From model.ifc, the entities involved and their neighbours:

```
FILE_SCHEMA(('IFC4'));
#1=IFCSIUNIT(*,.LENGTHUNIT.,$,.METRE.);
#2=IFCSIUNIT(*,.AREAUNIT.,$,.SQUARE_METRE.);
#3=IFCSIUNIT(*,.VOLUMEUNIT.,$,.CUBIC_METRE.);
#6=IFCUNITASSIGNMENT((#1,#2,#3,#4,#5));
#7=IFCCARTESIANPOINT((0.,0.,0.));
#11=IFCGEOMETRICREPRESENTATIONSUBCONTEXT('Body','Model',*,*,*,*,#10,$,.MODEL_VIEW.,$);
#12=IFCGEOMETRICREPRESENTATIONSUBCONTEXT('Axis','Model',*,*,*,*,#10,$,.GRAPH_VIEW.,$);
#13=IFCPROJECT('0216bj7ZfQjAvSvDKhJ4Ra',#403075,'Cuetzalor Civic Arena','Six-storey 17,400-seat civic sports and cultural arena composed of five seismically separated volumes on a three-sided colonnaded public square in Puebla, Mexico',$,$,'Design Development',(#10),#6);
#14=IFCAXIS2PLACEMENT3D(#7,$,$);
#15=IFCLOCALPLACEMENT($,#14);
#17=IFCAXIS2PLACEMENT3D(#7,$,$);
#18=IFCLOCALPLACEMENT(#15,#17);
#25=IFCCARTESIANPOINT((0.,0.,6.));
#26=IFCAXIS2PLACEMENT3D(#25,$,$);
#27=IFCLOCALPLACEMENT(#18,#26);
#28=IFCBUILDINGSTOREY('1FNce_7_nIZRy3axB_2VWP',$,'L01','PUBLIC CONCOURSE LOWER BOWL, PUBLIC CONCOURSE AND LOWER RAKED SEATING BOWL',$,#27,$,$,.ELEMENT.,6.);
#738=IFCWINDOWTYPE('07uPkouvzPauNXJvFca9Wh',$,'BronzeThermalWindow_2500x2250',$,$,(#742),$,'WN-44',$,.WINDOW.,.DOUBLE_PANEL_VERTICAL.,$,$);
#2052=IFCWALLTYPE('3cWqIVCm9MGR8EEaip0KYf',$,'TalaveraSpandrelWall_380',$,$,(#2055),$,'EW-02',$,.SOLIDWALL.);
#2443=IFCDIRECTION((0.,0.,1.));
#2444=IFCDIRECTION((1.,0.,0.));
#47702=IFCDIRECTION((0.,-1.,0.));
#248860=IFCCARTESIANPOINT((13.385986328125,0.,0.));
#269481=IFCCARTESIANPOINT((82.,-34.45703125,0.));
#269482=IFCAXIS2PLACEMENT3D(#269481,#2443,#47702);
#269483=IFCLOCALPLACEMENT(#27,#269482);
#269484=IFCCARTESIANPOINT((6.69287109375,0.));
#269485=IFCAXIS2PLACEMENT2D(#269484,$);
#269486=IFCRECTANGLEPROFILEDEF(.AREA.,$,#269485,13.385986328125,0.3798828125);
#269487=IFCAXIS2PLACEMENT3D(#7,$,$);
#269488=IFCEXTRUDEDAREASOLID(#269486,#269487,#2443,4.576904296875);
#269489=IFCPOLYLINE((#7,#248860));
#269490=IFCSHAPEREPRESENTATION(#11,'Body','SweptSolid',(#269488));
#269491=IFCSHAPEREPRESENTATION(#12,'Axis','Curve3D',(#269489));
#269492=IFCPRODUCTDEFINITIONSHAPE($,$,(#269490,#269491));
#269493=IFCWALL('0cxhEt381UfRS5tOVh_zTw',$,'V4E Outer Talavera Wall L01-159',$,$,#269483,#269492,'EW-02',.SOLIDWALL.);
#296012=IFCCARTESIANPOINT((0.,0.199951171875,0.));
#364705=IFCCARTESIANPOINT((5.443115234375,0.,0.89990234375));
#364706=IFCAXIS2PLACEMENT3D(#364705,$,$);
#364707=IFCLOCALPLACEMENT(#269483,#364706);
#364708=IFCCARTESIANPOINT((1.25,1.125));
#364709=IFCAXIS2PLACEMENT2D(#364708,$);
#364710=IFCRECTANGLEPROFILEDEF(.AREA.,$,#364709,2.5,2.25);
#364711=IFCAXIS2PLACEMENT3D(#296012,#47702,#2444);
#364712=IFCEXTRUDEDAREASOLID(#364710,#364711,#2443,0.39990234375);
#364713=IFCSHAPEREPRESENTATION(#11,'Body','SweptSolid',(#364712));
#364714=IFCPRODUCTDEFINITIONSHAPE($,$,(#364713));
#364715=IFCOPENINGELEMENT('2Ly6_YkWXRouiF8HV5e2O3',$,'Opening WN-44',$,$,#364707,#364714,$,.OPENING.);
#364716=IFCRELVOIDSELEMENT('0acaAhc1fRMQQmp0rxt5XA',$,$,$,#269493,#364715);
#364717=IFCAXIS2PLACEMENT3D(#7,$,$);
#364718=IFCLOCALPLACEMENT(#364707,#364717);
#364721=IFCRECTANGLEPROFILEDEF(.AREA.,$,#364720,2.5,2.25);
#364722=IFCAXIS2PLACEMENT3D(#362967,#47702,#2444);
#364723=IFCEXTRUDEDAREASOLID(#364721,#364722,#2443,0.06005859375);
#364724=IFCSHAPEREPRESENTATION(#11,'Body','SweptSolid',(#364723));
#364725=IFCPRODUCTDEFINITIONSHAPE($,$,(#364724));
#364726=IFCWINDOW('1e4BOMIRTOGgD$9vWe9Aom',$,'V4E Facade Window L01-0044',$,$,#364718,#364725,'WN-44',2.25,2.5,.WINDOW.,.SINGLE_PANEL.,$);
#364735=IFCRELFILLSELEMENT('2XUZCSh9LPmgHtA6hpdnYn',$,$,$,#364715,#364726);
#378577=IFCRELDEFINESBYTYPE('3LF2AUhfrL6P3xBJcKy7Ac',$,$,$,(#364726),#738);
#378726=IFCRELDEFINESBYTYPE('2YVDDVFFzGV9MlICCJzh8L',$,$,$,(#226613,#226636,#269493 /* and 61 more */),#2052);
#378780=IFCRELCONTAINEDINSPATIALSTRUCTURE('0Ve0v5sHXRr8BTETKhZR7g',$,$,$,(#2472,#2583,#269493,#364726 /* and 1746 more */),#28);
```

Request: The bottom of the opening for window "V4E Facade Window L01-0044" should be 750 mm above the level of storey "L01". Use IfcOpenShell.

```python
import numpy as np
import ifcopenshell
import ifcopenshell.api.geometry
import ifcopenshell.geom
import ifcopenshell.util.element
import ifcopenshell.util.placement
import ifcopenshell.util.shape
import ifcopenshell.util.unit

model = ifcopenshell.open("model.ifc")
unit_scale = ifcopenshell.util.unit.calculate_unit_scale(model)

window = model.by_guid("1e4BOMIRTOGgD$9vWe9Aom")
opening = window.FillsVoids[0].RelatingOpeningElement
storey = ifcopenshell.util.element.get_container(window, ifc_class="IfcBuildingStorey")
level = ifcopenshell.util.placement.get_local_placement(storey.ObjectPlacement)[2, 3]

# The opening's origin need not be at the sill, so measure its lowest point.
shape = ifcopenshell.geom.create_shape(ifcopenshell.geom.settings(), opening)
bottom = ifcopenshell.util.shape.get_shape_bottom_elevation(shape, shape.geometry) / unit_scale
dz = level + 0.75 / unit_scale - bottom

shift = np.array([0.0, 0.0, dz])
# The window is placed relative to its opening, so it follows when the opening moves.
matrix = ifcopenshell.util.placement.get_local_placement(opening.ObjectPlacement)
matrix[:3, 3] += shift
ifcopenshell.api.geometry.edit_object_placement(
    model, product=opening, matrix=matrix, is_si=False, should_transform_children=True
)

print(f"moved by {dz * unit_scale:+.3f} m")

model.write("model_rev.ifc")
```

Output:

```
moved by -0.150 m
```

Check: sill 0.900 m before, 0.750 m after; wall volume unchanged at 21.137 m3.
